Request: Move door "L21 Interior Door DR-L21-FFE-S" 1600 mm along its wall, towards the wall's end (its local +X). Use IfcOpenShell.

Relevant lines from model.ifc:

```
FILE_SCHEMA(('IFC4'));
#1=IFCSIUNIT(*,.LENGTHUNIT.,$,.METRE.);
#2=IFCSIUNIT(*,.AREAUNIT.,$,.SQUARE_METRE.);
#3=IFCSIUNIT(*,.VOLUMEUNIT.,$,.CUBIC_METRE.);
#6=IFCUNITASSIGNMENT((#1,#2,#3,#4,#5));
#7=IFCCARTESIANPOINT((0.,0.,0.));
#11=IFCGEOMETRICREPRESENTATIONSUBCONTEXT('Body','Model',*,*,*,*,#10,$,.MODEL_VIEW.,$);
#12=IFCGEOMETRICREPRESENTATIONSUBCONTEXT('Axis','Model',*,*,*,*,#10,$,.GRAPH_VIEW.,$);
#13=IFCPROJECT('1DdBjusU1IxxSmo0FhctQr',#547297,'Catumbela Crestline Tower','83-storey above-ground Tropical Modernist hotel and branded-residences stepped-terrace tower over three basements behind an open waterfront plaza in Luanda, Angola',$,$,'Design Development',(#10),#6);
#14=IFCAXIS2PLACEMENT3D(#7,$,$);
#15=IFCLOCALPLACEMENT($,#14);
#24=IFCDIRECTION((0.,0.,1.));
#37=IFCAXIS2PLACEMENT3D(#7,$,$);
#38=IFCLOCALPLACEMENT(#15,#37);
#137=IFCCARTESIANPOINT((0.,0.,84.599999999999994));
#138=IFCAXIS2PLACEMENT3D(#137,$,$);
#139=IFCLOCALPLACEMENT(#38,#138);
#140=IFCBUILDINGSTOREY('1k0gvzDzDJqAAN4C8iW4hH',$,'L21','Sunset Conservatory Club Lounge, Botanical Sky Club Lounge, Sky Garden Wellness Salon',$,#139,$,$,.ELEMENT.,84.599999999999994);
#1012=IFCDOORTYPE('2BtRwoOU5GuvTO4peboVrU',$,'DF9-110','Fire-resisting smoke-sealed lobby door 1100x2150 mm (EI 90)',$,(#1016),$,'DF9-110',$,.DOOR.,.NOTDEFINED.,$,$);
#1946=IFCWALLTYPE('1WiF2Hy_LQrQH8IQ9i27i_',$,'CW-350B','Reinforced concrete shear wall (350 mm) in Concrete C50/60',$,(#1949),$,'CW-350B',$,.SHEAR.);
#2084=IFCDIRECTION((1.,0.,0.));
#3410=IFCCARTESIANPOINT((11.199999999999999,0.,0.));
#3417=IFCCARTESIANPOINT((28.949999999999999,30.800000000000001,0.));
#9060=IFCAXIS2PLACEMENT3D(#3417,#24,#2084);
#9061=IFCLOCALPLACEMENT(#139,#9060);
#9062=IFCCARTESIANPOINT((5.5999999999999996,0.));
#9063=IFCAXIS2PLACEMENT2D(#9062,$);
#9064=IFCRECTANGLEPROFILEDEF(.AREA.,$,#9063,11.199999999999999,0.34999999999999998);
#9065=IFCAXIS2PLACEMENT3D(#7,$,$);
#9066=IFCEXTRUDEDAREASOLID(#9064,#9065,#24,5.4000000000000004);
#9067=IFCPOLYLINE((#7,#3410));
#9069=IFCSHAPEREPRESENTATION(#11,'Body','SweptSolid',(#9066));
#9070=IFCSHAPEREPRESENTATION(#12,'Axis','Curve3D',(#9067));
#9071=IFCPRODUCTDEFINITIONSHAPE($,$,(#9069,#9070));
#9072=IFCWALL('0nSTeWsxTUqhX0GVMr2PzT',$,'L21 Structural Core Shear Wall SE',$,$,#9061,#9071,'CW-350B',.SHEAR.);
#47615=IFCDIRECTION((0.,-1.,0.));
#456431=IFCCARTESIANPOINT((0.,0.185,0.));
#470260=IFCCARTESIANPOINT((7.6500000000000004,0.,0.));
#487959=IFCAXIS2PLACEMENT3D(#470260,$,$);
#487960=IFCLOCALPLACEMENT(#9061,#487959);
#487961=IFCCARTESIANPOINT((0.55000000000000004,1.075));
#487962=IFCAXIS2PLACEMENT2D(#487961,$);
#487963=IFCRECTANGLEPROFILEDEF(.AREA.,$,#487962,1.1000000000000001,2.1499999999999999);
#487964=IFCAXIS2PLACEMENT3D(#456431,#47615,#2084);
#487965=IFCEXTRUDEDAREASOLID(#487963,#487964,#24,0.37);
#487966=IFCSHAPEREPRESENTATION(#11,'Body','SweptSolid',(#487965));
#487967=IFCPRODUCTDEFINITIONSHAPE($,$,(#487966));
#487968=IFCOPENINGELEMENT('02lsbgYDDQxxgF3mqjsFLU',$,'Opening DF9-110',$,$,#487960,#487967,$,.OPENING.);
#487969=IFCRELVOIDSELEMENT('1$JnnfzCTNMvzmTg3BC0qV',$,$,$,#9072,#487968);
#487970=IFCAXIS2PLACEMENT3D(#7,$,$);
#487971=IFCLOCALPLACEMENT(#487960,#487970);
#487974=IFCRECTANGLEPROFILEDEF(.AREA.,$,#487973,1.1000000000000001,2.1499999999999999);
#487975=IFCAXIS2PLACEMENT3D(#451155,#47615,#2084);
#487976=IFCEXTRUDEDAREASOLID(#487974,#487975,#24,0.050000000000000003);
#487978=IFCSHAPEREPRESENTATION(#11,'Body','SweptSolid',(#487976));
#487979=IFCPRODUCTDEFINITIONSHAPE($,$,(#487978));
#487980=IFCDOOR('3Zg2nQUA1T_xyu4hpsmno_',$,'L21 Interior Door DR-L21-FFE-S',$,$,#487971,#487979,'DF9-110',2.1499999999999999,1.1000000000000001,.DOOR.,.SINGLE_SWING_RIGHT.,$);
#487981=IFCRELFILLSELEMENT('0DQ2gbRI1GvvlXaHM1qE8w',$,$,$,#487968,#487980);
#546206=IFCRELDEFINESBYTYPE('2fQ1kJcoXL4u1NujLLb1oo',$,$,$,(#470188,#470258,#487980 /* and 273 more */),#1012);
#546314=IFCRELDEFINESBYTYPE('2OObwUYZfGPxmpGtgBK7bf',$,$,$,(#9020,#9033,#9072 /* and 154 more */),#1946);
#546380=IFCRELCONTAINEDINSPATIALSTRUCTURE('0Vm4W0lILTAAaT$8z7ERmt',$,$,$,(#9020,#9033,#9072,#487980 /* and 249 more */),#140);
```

```python
import ifcopenshell
import ifcopenshell.api.geometry
import ifcopenshell.util.placement

model = ifcopenshell.open("model.ifc")

door = model.by_id(487980)
opening = door.FillsVoids[0].RelatingOpeningElement
wall = opening.VoidsElements[0].RelatingBuildingElement

wall_matrix = ifcopenshell.util.placement.get_local_placement(wall.ObjectPlacement)
shift = wall_matrix[:3, 0] * 1.6
before = ifcopenshell.util.placement.get_local_placement(door.ObjectPlacement)[:3, 3].copy()

# The door is placed relative to its opening, so it follows when the opening moves.
matrix = ifcopenshell.util.placement.get_local_placement(opening.ObjectPlacement)
matrix[:3, 3] += shift
ifcopenshell.api.geometry.edit_object_placement(
    model, product=opening, matrix=matrix, is_si=False, should_transform_children=True
)

after = ifcopenshell.util.placement.get_local_placement(door.ObjectPlacement)[:3, 3]
print("door moved by", (after - before).round(3) + 0.0)

model.write("model_updated.ifc")
```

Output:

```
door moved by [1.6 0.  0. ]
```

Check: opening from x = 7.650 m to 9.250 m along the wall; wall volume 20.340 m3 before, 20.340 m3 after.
